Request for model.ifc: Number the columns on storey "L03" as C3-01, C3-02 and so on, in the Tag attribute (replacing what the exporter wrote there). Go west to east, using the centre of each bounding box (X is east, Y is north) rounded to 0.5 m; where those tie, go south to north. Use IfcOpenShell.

First a look at what the model holds.

```python
import ifcopenshell
import ifcopenshell.util.element
import ifcopenshell.util.placement

model = ifcopenshell.open("model.ifc")
print(model.schema)
storey = next(s for s in model.by_type("IfcBuildingStorey") if s.Name == "L03")
columns = [e for e in ifcopenshell.util.element.get_decomposition(storey) if e.is_a("IfcColumn")]
for e in sorted(columns, key=lambda e: e.id()):
    origin = ifcopenshell.util.placement.get_local_placement(e.ObjectPlacement)[:3, 3]
    print(e.id(), e.Tag, e.Name, origin.round(2) + 0.0, sep=" | ")
```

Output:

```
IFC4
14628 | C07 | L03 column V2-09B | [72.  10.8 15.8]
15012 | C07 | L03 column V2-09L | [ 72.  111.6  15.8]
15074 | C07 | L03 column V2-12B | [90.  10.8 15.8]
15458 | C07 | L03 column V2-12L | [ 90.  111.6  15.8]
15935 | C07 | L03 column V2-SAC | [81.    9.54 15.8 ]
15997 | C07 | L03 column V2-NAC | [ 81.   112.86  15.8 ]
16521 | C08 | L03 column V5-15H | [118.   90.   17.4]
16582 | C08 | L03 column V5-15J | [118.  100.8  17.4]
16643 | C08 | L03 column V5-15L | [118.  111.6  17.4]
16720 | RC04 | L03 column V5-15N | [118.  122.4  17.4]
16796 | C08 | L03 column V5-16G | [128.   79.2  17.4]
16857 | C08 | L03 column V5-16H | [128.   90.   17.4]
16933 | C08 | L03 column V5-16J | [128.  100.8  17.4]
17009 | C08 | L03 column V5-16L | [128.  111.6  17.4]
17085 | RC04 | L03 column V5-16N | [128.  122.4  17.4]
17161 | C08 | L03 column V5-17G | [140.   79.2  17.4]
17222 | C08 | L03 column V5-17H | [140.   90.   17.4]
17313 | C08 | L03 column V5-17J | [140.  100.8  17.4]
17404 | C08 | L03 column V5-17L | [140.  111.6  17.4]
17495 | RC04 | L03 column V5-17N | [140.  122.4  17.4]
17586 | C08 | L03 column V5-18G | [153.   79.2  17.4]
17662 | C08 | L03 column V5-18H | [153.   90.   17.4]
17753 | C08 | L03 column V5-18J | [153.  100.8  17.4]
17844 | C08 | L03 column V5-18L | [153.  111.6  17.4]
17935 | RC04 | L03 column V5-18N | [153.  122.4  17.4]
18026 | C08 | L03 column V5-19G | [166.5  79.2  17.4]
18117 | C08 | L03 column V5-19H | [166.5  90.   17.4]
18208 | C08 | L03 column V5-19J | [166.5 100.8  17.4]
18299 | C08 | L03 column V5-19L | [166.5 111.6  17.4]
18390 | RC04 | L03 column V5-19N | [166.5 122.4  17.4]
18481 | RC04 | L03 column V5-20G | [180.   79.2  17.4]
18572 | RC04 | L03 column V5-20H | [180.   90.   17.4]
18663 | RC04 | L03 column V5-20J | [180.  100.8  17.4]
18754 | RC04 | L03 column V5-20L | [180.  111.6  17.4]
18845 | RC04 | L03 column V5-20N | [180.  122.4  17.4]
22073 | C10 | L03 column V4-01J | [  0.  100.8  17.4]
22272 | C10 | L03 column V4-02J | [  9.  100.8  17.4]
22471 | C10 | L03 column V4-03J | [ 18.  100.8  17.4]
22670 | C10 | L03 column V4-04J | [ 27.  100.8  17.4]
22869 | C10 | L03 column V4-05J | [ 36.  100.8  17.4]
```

```python
import ifcopenshell
import ifcopenshell.geom
import ifcopenshell.util.element
import ifcopenshell.util.shape

model = ifcopenshell.open("model.ifc")
settings = ifcopenshell.geom.settings()
settings.set("use-world-coords", True)


def centre(element):
    shape = ifcopenshell.geom.create_shape(settings, element)
    return ifcopenshell.util.shape.get_bbox_centroid(shape.geometry)


storey = next(s for s in model.by_type("IfcBuildingStorey") if s.Name == "L03")
columns = [e for e in ifcopenshell.util.element.get_decomposition(storey) if e.is_a("IfcColumn")]

# Insertion points can sit at a corner or the storey origin, so sort by the geometry (in metres).
centres = {e: centre(e) for e in columns}
columns.sort(key=lambda e: (round(centres[e][0] / 0.5), centres[e][1]))

for i, e in enumerate(columns, start=1):
    number = f"C3-{i:02d}"
    e.Tag = number
    print(e.id(), number)

model.write("model_rev.ifc")
```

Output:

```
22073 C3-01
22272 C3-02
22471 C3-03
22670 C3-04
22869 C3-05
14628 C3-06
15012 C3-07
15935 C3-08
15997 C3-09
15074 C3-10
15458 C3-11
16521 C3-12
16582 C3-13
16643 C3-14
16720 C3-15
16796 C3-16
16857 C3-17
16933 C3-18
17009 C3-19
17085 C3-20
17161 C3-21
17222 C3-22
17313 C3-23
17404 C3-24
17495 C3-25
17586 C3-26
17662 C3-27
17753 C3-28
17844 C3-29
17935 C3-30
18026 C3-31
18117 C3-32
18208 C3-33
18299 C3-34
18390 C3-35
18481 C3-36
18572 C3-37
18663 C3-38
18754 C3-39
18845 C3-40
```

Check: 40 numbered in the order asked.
